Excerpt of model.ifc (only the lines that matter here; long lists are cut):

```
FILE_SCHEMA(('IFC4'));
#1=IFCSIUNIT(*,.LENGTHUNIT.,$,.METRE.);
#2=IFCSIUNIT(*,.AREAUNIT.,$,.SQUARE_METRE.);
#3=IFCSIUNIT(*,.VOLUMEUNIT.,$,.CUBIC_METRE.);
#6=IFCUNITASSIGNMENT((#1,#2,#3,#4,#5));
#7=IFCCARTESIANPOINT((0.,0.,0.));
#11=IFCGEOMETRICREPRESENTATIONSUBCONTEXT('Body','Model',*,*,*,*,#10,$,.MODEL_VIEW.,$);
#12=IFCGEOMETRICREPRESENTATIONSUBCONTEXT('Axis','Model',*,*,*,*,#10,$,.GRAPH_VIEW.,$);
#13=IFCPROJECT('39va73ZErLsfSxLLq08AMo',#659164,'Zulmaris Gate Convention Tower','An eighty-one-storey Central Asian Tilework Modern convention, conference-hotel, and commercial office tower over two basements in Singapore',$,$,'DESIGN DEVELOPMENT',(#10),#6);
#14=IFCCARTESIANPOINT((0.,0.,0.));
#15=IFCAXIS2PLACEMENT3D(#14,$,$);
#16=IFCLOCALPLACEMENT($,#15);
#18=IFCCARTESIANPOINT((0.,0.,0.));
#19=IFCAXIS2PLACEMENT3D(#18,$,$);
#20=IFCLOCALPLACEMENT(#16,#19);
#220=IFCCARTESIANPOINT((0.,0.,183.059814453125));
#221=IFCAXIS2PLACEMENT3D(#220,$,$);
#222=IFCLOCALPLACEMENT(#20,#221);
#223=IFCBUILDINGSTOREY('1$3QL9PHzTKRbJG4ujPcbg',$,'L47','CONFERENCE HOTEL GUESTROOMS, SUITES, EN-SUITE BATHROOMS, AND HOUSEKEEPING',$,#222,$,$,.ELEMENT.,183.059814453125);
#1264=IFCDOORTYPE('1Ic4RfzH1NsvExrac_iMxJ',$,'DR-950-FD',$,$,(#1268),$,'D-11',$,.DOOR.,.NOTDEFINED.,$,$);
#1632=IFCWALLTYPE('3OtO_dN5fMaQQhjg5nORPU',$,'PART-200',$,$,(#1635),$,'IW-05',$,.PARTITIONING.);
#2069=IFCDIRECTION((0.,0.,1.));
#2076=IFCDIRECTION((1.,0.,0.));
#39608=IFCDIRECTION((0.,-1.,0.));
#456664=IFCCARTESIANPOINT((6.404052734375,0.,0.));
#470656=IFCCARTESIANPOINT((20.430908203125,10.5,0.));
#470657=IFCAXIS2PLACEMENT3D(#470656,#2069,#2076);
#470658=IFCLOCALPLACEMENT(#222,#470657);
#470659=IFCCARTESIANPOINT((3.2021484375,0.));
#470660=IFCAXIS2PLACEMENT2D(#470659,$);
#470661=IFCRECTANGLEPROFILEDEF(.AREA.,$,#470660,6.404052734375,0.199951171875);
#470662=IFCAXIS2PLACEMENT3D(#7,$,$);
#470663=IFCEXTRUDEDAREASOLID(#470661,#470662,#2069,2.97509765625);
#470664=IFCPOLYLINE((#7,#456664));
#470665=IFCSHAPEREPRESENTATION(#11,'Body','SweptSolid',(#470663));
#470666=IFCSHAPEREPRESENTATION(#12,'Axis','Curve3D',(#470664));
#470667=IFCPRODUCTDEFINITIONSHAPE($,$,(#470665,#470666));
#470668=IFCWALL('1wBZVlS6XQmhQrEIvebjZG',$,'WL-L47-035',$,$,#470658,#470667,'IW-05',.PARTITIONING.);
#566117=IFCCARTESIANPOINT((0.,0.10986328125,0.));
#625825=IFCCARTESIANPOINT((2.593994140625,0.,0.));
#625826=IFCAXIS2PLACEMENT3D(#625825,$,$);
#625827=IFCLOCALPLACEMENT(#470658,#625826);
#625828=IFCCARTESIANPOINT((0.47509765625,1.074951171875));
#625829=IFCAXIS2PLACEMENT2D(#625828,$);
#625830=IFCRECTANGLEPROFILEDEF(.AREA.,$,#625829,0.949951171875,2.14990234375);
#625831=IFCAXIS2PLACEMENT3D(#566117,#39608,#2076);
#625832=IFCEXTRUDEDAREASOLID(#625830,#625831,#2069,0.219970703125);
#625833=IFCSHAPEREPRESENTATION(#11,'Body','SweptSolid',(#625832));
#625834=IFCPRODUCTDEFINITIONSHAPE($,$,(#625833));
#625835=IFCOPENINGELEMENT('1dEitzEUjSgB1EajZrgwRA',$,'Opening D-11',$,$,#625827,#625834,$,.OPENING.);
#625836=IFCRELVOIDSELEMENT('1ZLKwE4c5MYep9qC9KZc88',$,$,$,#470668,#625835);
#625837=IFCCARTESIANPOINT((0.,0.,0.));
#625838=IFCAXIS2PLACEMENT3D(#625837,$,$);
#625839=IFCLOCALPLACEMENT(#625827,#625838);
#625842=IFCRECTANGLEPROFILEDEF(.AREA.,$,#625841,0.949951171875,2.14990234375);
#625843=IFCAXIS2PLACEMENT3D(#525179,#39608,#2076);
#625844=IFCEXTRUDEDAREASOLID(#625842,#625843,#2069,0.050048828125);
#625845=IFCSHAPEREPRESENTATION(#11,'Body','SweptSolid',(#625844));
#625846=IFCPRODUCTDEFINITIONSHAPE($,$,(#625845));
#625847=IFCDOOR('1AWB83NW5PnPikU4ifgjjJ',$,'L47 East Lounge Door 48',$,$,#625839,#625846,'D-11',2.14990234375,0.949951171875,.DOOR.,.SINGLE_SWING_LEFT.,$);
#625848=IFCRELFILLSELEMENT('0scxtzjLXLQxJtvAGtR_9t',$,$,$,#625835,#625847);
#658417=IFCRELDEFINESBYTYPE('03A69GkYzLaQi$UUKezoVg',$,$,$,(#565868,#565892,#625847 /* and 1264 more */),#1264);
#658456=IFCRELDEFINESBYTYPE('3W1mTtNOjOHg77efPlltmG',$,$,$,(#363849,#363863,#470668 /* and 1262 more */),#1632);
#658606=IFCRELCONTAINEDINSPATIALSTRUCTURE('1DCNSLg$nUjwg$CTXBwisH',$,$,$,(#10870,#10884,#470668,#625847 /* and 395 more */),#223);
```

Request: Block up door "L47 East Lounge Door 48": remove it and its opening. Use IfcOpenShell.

```python
import ifcopenshell
import ifcopenshell.api.feature
import ifcopenshell.api.root
import ifcopenshell.geom
import ifcopenshell.util.shape

model = ifcopenshell.open("model.ifc")
settings = ifcopenshell.geom.settings()


def volume(element):
    """Net volume in cubic metres, openings subtracted."""
    shape = ifcopenshell.geom.create_shape(settings, element)
    return ifcopenshell.util.shape.get_volume(shape.geometry)


door = model.by_guid("1AWB83NW5PnPikU4ifgjjJ")
opening = door.FillsVoids[0].RelatingOpeningElement
wall = opening.VoidsElements[0].RelatingBuildingElement
before = volume(wall)

ifcopenshell.api.root.remove_product(model, product=door)
ifcopenshell.api.feature.remove_feature(model, feature=opening)

after = volume(wall)

print(f"wall volume {before:.3f} -> {after:.3f} m3")

model.write("model_rev.ifc")
```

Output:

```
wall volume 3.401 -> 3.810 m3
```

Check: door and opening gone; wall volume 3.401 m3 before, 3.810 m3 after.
